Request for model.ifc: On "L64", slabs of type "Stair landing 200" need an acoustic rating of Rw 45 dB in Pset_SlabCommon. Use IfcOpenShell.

First a look at what the model holds.

```python
import ifcopenshell
import ifcopenshell.util.element

model = ifcopenshell.open("model.ifc")
print(model.schema)
storey = next(s for s in model.by_type("IfcBuildingStorey") if s.Name == "L64")
slabs = [e for e in ifcopenshell.util.element.get_decomposition(storey) if e.is_a("IfcSlab")]
seen = {}
for e in slabs:
    element_type = ifcopenshell.util.element.get_type(e)
    key = (element_type.Name if element_type != e and element_type else None, ifcopenshell.util.element.get_pset(e, "Pset_SlabCommon", "AcousticRating"))
    seen[key] = seen.get(key, 0) + 1
for (name, value), count in sorted(seen.items(), key=str):
    print(count, "x", name, "|", value)
```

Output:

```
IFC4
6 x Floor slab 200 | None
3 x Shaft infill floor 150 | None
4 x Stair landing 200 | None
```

```python
import ifcopenshell
import ifcopenshell.api.pset
import ifcopenshell.util.element

model = ifcopenshell.open("model.ifc")

storey = next(s for s in model.by_type("IfcBuildingStorey") if s.Name == "L64")
slabs = [e for e in ifcopenshell.util.element.get_decomposition(storey) if e.is_a("IfcSlab")]

count = 0
for e in slabs:
    element_type = ifcopenshell.util.element.get_type(e)
    if element_type in (None, e) or element_type.Name != "Stair landing 200":
        continue
    found = ifcopenshell.util.element.get_pset(e, "Pset_SlabCommon", should_inherit=False)
    if found:
        pset = model.by_id(found["id"])
        if len(ifcopenshell.util.element.get_elements_by_pset(pset)) > 1:
            pset = ifcopenshell.api.pset.unshare_pset(model, products=[e], pset=pset)[0]
    else:
        pset = ifcopenshell.api.pset.add_pset(model, product=e, name="Pset_SlabCommon")
    ifcopenshell.api.pset.edit_pset(model, pset=pset, properties={"AcousticRating": "Rw 45 dB"})
    count += 1

print(count, "slabs updated")

model.write("model_updated.ifc")
```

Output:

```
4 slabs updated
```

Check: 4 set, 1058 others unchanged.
